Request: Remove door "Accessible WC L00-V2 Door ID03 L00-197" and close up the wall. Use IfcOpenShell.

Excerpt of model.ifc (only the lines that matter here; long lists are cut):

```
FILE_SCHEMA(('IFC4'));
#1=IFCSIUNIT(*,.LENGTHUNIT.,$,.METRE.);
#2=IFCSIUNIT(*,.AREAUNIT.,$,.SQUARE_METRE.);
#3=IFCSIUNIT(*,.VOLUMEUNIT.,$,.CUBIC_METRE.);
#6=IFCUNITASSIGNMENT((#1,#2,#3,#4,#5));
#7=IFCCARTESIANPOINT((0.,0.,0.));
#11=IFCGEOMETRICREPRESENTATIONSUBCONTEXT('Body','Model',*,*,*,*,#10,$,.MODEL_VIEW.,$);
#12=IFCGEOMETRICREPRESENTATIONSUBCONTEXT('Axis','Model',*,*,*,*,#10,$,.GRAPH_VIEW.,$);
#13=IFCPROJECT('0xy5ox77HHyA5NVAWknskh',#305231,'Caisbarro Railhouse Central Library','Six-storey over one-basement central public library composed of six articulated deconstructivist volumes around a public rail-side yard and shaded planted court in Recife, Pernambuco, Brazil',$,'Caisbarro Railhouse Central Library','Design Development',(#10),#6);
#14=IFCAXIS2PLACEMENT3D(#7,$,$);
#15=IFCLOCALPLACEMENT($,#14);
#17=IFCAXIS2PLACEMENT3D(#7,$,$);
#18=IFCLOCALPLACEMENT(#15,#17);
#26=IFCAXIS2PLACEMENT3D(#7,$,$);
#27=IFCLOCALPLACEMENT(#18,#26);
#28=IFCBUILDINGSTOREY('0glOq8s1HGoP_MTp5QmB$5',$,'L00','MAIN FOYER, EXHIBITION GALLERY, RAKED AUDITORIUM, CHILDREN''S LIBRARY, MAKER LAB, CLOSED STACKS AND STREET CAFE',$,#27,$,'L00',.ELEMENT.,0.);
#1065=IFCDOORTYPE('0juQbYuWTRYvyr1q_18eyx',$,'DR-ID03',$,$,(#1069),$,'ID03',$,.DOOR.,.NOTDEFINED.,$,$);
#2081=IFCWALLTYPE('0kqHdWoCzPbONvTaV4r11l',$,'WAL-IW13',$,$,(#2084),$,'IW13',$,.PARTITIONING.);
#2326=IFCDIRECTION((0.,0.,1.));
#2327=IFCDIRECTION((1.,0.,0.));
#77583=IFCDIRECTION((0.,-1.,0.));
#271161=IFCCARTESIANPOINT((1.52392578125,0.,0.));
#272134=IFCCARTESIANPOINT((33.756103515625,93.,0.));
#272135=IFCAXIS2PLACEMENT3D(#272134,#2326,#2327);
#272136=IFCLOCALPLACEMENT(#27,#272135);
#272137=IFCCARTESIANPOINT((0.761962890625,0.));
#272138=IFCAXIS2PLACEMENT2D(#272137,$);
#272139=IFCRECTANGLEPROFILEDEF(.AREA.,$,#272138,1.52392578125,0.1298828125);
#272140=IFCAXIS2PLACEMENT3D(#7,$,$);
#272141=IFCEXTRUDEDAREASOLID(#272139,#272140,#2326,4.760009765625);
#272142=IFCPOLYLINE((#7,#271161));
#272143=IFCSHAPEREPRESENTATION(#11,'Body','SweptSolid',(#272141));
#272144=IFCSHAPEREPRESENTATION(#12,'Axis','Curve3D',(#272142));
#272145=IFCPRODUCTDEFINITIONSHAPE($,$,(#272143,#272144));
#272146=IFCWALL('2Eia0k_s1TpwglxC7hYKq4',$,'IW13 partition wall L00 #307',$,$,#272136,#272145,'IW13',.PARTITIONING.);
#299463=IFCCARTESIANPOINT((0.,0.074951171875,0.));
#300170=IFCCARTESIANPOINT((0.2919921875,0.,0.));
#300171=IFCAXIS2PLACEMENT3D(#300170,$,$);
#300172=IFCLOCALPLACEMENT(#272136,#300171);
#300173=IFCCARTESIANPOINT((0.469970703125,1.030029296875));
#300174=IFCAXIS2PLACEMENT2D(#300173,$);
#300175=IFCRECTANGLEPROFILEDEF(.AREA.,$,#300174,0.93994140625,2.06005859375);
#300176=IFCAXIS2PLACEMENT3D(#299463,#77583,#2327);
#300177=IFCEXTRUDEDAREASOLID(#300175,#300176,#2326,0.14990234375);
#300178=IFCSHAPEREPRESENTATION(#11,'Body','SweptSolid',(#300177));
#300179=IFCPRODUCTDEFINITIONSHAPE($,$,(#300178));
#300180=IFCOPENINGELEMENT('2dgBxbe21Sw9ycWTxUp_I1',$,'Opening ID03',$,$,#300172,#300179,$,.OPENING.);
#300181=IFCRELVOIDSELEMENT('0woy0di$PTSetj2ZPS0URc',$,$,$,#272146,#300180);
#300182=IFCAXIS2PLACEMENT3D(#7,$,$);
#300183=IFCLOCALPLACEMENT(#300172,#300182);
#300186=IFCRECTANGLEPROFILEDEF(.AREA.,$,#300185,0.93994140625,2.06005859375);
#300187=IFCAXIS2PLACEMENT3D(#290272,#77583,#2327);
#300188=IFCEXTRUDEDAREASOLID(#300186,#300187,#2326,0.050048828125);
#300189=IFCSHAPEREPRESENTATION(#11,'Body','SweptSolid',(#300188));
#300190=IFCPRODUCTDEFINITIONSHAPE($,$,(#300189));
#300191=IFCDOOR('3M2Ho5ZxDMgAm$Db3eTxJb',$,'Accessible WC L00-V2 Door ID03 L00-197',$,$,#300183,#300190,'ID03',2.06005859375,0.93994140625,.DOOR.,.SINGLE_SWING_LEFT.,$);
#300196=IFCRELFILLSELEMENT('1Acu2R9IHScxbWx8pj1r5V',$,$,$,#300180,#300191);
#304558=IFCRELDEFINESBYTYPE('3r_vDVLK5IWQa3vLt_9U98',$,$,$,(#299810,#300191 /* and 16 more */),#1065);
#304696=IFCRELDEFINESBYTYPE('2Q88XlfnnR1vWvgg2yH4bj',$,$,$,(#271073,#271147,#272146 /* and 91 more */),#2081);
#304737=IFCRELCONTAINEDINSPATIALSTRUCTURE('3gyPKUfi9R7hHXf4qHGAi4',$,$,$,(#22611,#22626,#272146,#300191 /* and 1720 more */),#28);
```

```python
import ifcopenshell
import ifcopenshell.api.feature
import ifcopenshell.api.root
import ifcopenshell.geom
import ifcopenshell.util.shape

model = ifcopenshell.open("model.ifc")
settings = ifcopenshell.geom.settings()


def volume(element):
    """Net volume in cubic metres, openings subtracted."""
    shape = ifcopenshell.geom.create_shape(settings, element)
    return ifcopenshell.util.shape.get_volume(shape.geometry)


door = model.by_id(300191)
opening = door.FillsVoids[0].RelatingOpeningElement
wall = opening.VoidsElements[0].RelatingBuildingElement
before = volume(wall)

ifcopenshell.api.root.remove_product(model, product=door)
ifcopenshell.api.feature.remove_feature(model, feature=opening)

after = volume(wall)

print(f"wall volume {before:.3f} -> {after:.3f} m3")

model.write("model_v2.ifc")
```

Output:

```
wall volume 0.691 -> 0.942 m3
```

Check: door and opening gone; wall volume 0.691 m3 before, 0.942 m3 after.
